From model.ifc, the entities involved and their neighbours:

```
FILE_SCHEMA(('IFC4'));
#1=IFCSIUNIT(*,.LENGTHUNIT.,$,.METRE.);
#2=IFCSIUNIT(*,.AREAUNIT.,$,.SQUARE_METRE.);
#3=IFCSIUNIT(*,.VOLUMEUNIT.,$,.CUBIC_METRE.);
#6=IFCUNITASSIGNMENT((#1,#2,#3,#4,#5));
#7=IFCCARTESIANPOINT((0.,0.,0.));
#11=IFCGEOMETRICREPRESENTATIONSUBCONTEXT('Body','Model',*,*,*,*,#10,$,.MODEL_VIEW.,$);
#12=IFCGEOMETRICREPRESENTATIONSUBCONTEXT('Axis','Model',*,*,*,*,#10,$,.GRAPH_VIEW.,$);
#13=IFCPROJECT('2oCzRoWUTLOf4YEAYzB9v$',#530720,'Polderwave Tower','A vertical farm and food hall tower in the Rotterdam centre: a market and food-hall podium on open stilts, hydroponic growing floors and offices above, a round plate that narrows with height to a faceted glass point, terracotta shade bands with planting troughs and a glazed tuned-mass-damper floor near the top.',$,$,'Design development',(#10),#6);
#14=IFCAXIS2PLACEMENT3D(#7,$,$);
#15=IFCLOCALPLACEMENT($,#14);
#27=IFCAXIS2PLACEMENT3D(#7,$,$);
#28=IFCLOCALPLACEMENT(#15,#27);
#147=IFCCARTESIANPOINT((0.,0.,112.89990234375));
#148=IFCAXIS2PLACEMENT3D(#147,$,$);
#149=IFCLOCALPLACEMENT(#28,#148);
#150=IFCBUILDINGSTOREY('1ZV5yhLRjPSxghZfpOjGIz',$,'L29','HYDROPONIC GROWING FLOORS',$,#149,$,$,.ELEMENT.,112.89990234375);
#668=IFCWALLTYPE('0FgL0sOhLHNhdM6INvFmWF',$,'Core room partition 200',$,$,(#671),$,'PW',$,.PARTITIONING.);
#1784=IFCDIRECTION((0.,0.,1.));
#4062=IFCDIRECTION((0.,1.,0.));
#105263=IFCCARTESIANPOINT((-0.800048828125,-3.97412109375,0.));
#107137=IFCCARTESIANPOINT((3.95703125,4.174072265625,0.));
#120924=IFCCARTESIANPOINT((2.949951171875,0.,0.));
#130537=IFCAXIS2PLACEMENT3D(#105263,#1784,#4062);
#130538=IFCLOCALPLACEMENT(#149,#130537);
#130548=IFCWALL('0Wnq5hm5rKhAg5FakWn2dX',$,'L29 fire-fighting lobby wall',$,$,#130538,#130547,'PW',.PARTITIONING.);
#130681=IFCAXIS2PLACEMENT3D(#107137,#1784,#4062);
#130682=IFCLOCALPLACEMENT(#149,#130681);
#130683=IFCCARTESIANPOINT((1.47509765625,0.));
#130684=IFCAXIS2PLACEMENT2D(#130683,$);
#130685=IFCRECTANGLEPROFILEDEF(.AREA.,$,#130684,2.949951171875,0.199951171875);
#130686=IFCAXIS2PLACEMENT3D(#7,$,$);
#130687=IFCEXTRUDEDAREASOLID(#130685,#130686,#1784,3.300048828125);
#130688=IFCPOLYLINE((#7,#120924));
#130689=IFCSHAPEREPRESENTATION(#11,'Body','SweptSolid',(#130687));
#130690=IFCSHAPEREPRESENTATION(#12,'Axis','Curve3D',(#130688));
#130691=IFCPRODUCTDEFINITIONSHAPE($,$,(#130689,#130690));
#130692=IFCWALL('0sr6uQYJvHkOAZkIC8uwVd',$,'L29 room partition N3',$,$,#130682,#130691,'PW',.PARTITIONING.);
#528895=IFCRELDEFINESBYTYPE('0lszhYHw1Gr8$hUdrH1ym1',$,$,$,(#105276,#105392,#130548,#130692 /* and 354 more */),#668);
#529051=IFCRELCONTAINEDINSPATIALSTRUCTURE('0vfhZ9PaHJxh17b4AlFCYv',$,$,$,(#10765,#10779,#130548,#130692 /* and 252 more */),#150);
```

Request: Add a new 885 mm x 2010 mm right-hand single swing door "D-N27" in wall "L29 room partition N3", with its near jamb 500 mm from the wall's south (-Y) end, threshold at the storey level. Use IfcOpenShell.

```python
import numpy as np
import ifcopenshell
import ifcopenshell.api.feature
import ifcopenshell.api.geometry
import ifcopenshell.api.root
import ifcopenshell.api.spatial
import ifcopenshell.geom
import ifcopenshell.util.element
import ifcopenshell.util.placement
import ifcopenshell.util.representation
import ifcopenshell.util.shape
import ifcopenshell.util.unit

model = ifcopenshell.open("model.ifc")
unit_scale = ifcopenshell.util.unit.calculate_unit_scale(model)
settings = ifcopenshell.geom.settings()


def volume(element):
    """Net volume in cubic metres, openings subtracted."""
    shape = ifcopenshell.geom.create_shape(settings, element)
    return ifcopenshell.util.shape.get_volume(shape.geometry)


wall = model.by_guid("0sr6uQYJvHkOAZkIC8uwVd")
storey = ifcopenshell.util.element.get_container(wall, ifc_class="IfcBuildingStorey")
context = ifcopenshell.util.representation.get_context(model, "Model", "Body", "MODEL_VIEW")
before = volume(wall)

width, height, from_end, sill = 0.885, 2.01, 0.5, 0.0  # metres

# The wall runs along its own X axis, and the end named is its -X end.
wall_shape = ifcopenshell.geom.create_shape(settings, wall)
x, y, z = ifcopenshell.util.shape.get_vertices(wall_shape.geometry).T
start = x.min() + from_end
face, thickness = float(y.min()), float(y.max() - y.min())
wall_matrix = ifcopenshell.util.placement.get_local_placement(wall.ObjectPlacement)
level = ifcopenshell.util.placement.get_local_placement(storey.ObjectPlacement)[2, 3]


def in_wall(x, y):
    """Placement at x, y metres in the wall's axes, at sill height."""
    matrix = wall_matrix.copy()
    matrix[:, 3] = wall_matrix @ np.array([x / unit_scale, y / unit_scale, 0.0, 1.0])
    matrix[2, 3] = level + sill / unit_scale
    return matrix


# Opening: a box that overshoots both wall faces by 50 mm.
opening = ifcopenshell.api.root.create_entity(model, ifc_class="IfcOpeningElement", predefined_type="OPENING")
box = ifcopenshell.api.geometry.add_wall_representation(
    model, context=context, length=width, height=height, thickness=thickness + 0.1
)
ifcopenshell.api.geometry.assign_representation(model, product=opening, representation=box)
ifcopenshell.api.geometry.edit_object_placement(model, product=opening, matrix=in_wall(start, face - 0.05), is_si=False)
ifcopenshell.api.feature.add_feature(model, feature=opening, element=wall)

door = ifcopenshell.api.root.create_entity(model, ifc_class="IfcDoor", name="D-N27", predefined_type="DOOR")
door.OverallWidth, door.OverallHeight = width / unit_scale, height / unit_scale
door.OperationType = "SINGLE_SWING_RIGHT"
body = ifcopenshell.api.geometry.add_door_representation(
    model,
    context=context,
    overall_width=door.OverallWidth,
    overall_height=door.OverallHeight,
    operation_type="SINGLE_SWING_RIGHT",
    lining_properties={"LiningDepth": thickness / unit_scale, "ThresholdDepth": thickness / unit_scale},
)
ifcopenshell.api.geometry.assign_representation(model, product=door, representation=body)
ifcopenshell.api.spatial.assign_container(model, products=[door], relating_structure=storey)
ifcopenshell.api.feature.add_filling(model, opening=opening, element=door)

# The lining spans the wall, so the door starts at the wall face.
ifcopenshell.api.geometry.edit_object_placement(model, product=door, matrix=in_wall(start, face), is_si=False)

after = volume(wall)

print(f"wall volume {before:.3f} -> {after:.3f} m3")

model.write("model_rev.ifc")
```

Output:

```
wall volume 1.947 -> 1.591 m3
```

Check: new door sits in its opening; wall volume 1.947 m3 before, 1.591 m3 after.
